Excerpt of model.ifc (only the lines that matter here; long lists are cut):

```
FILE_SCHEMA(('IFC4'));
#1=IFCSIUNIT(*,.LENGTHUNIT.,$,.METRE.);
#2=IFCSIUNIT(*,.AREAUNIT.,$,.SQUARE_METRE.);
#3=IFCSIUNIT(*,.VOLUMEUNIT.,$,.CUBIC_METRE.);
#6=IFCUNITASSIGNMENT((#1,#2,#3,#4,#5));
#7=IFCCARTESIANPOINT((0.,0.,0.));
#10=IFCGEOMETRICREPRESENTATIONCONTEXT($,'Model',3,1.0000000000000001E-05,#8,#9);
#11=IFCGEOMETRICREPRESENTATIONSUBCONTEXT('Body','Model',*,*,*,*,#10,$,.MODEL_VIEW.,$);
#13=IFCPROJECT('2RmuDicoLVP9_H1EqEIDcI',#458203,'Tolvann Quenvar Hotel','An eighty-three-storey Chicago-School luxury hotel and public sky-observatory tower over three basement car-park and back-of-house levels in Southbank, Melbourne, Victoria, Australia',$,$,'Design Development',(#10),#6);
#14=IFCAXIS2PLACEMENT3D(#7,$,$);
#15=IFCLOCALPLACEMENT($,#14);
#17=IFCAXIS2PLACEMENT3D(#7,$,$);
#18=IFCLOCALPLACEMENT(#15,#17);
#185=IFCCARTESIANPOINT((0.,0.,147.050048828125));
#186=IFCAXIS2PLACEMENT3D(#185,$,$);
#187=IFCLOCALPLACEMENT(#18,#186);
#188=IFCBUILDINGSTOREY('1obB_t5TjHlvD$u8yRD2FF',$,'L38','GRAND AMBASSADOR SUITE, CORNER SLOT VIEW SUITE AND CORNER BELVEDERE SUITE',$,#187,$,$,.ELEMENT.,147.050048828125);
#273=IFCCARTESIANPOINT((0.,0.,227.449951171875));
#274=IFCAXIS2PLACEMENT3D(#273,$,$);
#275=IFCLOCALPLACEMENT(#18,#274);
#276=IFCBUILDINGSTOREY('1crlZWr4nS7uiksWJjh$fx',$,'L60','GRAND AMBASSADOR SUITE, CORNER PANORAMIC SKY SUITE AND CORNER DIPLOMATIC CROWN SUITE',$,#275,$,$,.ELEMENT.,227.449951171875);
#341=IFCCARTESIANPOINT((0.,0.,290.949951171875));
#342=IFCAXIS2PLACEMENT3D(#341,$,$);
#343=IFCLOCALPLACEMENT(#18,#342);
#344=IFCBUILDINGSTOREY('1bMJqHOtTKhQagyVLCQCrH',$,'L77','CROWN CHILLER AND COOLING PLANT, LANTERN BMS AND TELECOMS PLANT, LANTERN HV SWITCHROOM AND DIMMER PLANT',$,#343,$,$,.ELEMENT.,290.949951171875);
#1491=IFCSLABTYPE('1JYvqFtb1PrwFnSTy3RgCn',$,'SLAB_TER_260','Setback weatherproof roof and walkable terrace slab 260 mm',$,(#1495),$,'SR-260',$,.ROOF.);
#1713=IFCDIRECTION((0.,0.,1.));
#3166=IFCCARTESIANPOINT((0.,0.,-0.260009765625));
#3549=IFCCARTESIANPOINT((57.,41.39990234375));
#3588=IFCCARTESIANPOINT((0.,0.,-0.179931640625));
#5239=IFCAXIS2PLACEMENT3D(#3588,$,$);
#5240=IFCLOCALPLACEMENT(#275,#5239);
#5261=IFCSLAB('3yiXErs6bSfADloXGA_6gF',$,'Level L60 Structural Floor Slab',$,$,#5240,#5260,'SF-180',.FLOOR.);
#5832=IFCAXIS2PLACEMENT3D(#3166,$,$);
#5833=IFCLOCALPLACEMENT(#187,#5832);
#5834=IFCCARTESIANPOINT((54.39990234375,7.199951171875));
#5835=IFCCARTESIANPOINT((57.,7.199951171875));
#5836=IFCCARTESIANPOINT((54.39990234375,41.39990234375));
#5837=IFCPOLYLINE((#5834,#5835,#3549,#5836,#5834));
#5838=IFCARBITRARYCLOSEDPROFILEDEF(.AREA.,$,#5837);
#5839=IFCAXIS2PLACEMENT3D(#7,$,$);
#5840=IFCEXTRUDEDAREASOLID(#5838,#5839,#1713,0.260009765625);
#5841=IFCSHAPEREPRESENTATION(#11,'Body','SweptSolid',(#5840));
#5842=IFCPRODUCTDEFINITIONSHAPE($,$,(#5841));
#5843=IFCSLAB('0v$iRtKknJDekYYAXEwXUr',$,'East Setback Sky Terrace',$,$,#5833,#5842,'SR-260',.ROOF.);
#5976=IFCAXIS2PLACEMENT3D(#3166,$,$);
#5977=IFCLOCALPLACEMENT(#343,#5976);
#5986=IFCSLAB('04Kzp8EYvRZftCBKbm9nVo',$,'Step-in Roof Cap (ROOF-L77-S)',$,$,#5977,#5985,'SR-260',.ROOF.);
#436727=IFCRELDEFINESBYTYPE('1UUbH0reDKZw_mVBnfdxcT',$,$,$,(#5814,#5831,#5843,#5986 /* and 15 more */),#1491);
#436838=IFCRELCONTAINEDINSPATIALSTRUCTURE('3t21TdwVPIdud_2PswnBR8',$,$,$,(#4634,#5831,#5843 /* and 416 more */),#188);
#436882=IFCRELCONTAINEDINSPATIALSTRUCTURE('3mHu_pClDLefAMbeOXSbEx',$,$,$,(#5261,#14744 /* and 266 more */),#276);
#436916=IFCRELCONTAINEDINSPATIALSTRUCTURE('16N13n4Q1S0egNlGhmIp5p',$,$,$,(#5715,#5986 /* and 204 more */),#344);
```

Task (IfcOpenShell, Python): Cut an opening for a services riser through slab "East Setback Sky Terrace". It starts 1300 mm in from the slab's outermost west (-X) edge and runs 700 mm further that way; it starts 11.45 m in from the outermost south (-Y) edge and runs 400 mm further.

```python
import numpy as np
import ifcopenshell
import ifcopenshell.api.feature
import ifcopenshell.api.geometry
import ifcopenshell.api.root
import ifcopenshell.geom
import ifcopenshell.util.placement
import ifcopenshell.util.representation
import ifcopenshell.util.shape
import ifcopenshell.util.unit

model = ifcopenshell.open("model.ifc")
unit_scale = ifcopenshell.util.unit.calculate_unit_scale(model)
settings = ifcopenshell.geom.settings()


def volume(element):
    """Net volume in cubic metres, openings subtracted."""
    shape = ifcopenshell.geom.create_shape(settings, element)
    return ifcopenshell.util.shape.get_volume(shape.geometry)


slab = model.by_guid("0v$iRtKknJDekYYAXEwXUr")
before = volume(slab)

# Extent in the slab's own axes, in metres. The edges named are its -X and -Y sides.
slab_shape = ifcopenshell.geom.create_shape(settings, slab)
vertices = ifcopenshell.util.shape.get_vertices(slab_shape.geometry)
x_min, y_min, bottom = vertices.min(axis=0)
top = vertices[:, 2].max()

opening = ifcopenshell.api.root.create_entity(model, ifc_class="IfcOpeningElement", name="Services riser opening", predefined_type="OPENING")
context = ifcopenshell.util.representation.get_context(model, "Model", "Body", "MODEL_VIEW")
width, depth = 0.7, 0.4
outline = [(0.0, 0.0), (width, 0.0), (width, depth), (0.0, depth), (0.0, 0.0)]
# Overshoot both faces by 50 mm so the cut is clean.
shape = ifcopenshell.api.geometry.add_slab_representation(
    model, context=context, depth=top - bottom + 0.1, polyline=outline
)
ifcopenshell.api.geometry.assign_representation(model, product=opening, representation=shape)

matrix = ifcopenshell.util.placement.get_local_placement(slab.ObjectPlacement)
matrix[:, 3] = matrix @ np.append(np.array([x_min + 1.3, y_min + 11.45, bottom - 0.05]) / unit_scale, 1.0)
ifcopenshell.api.geometry.edit_object_placement(model, product=opening, matrix=matrix, is_si=False)
ifcopenshell.api.feature.add_feature(model, feature=opening, element=slab)

after = volume(slab)

print(f"slab volume {before:.3f} -> {after:.3f} m3")

model.write("model_updated.ifc")
```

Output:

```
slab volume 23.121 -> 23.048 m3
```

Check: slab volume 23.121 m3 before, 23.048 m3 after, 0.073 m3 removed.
